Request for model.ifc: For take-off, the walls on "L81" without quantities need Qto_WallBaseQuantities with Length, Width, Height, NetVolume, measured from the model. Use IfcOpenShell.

First a look at what the model holds.

```python
import ifcopenshell
import ifcopenshell.util.element
import ifcopenshell.util.unit

model = ifcopenshell.open("model.ifc")
print(model.schema)
for unit_type in ("LENGTHUNIT", "AREAUNIT", "VOLUMEUNIT"):
    print(unit_type, ifcopenshell.util.unit.calculate_unit_scale(model, unit_type))
storey = next(s for s in model.by_type("IfcBuildingStorey") if s.Name == "L81")
walls = [e for e in ifcopenshell.util.element.get_decomposition(storey) if e.is_a("IfcWall")]
for e in sorted(walls, key=lambda e: e.id()):
    print(e.id(), e.is_a(), e.Name, list(ifcopenshell.util.element.get_psets(e, qtos_only=True)), sep=" | ")
```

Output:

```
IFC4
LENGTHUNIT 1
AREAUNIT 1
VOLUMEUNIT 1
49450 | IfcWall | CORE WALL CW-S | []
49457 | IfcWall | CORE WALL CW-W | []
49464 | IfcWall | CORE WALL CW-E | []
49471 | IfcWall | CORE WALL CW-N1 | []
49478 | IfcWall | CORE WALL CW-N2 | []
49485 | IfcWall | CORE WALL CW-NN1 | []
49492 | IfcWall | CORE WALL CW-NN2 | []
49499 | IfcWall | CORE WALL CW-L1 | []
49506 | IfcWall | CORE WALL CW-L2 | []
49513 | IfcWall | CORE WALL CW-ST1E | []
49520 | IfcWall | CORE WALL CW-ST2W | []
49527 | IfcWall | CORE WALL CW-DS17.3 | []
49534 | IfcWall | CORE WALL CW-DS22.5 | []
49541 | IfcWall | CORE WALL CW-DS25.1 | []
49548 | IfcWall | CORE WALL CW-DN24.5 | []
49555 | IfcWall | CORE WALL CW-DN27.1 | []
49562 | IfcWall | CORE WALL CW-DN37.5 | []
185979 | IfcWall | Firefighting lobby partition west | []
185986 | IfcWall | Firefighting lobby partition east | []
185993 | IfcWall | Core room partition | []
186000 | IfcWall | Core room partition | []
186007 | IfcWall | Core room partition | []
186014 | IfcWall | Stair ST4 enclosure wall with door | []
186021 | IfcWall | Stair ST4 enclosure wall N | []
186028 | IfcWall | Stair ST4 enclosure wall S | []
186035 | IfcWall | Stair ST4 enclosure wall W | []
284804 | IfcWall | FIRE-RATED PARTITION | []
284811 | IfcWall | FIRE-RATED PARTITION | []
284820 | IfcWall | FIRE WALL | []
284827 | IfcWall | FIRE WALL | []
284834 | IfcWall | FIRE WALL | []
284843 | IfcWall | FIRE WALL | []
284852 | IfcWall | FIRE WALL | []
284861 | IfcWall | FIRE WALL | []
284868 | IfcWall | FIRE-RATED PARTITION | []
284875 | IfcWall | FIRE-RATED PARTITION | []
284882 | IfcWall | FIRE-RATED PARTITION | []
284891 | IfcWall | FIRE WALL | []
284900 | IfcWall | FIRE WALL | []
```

```python
import ifcopenshell
import ifcopenshell.api.pset
import ifcopenshell.geom
import ifcopenshell.util.element
import ifcopenshell.util.shape
import ifcopenshell.util.unit

model = ifcopenshell.open("model.ifc")
unit_scale = ifcopenshell.util.unit.calculate_unit_scale(model)
volume_scale = ifcopenshell.util.unit.calculate_unit_scale(model, "VOLUMEUNIT")
settings = ifcopenshell.geom.settings()

storey = next(s for s in model.by_type("IfcBuildingStorey") if s.Name == "L81")
walls = [e for e in ifcopenshell.util.element.get_decomposition(storey) if e.is_a("IfcWall")]

for e in sorted(walls, key=lambda e: e.id()):
    if ifcopenshell.util.element.get_psets(e, qtos_only=True, should_inherit=False):
        continue
    # Geometry comes back in metres, in the element's own axes.
    shape = ifcopenshell.geom.create_shape(settings, e)
    values = {
        "Length": ifcopenshell.util.shape.get_x(shape.geometry) / unit_scale,
        "Width": ifcopenshell.util.shape.get_y(shape.geometry) / unit_scale,
        "Height": ifcopenshell.util.shape.get_z(shape.geometry) / unit_scale,
        "NetVolume": ifcopenshell.util.shape.get_volume(shape.geometry) / volume_scale,
    }
    qto = ifcopenshell.api.pset.add_qto(model, product=e, name="Qto_WallBaseQuantities")
    ifcopenshell.api.pset.edit_qto(model, qto=qto, properties=values)
    print(e.id(), {k: round(v, 3) for k, v in values.items()})

model.write("model_edited.ifc")
```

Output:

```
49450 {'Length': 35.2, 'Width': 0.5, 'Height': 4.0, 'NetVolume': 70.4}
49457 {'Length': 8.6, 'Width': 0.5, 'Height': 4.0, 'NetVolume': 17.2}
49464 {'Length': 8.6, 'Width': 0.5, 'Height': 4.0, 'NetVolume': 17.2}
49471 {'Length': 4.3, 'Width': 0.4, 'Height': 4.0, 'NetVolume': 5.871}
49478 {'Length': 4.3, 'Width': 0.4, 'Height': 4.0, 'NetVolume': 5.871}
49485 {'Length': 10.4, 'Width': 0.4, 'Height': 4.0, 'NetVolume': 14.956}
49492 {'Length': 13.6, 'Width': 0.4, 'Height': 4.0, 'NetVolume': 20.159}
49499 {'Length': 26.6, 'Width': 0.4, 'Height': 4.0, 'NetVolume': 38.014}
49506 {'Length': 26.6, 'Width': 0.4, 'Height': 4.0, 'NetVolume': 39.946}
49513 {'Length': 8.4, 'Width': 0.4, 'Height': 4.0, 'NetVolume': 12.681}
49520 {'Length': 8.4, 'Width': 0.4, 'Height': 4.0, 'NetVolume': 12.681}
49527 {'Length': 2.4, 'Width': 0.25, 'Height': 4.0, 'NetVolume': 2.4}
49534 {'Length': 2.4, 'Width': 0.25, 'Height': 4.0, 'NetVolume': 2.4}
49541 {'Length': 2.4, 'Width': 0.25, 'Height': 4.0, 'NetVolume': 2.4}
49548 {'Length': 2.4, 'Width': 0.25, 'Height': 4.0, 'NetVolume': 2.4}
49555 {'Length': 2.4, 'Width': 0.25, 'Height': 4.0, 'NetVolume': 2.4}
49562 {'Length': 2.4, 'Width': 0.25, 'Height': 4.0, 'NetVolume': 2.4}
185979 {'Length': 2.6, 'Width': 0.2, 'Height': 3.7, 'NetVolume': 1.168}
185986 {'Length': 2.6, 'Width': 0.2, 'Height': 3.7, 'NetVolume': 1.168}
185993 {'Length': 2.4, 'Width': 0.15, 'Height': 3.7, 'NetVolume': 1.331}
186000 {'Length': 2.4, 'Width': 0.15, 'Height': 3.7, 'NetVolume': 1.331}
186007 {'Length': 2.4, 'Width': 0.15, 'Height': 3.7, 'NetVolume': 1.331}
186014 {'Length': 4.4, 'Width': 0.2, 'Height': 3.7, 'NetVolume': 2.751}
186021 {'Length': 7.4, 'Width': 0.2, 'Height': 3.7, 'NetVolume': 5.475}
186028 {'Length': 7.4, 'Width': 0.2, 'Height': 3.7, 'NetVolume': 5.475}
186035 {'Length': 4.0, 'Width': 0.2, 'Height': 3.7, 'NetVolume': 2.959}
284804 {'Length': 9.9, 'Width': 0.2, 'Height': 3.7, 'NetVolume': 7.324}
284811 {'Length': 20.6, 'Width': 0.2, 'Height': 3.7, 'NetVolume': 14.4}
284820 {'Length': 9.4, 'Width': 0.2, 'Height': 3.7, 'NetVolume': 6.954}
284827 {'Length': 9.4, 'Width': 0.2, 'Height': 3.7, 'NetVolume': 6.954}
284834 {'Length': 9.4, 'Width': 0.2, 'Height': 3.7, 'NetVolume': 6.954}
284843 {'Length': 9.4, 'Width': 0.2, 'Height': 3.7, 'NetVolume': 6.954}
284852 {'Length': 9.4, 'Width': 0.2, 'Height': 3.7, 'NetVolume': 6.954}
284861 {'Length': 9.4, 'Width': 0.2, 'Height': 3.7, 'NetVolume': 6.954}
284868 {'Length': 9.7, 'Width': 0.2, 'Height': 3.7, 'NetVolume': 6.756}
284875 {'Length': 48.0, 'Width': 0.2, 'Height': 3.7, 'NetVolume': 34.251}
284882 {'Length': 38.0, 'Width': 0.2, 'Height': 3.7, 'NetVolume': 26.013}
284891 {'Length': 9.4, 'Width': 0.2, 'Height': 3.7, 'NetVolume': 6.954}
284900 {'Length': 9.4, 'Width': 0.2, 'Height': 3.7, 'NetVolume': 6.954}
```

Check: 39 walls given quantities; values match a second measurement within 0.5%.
